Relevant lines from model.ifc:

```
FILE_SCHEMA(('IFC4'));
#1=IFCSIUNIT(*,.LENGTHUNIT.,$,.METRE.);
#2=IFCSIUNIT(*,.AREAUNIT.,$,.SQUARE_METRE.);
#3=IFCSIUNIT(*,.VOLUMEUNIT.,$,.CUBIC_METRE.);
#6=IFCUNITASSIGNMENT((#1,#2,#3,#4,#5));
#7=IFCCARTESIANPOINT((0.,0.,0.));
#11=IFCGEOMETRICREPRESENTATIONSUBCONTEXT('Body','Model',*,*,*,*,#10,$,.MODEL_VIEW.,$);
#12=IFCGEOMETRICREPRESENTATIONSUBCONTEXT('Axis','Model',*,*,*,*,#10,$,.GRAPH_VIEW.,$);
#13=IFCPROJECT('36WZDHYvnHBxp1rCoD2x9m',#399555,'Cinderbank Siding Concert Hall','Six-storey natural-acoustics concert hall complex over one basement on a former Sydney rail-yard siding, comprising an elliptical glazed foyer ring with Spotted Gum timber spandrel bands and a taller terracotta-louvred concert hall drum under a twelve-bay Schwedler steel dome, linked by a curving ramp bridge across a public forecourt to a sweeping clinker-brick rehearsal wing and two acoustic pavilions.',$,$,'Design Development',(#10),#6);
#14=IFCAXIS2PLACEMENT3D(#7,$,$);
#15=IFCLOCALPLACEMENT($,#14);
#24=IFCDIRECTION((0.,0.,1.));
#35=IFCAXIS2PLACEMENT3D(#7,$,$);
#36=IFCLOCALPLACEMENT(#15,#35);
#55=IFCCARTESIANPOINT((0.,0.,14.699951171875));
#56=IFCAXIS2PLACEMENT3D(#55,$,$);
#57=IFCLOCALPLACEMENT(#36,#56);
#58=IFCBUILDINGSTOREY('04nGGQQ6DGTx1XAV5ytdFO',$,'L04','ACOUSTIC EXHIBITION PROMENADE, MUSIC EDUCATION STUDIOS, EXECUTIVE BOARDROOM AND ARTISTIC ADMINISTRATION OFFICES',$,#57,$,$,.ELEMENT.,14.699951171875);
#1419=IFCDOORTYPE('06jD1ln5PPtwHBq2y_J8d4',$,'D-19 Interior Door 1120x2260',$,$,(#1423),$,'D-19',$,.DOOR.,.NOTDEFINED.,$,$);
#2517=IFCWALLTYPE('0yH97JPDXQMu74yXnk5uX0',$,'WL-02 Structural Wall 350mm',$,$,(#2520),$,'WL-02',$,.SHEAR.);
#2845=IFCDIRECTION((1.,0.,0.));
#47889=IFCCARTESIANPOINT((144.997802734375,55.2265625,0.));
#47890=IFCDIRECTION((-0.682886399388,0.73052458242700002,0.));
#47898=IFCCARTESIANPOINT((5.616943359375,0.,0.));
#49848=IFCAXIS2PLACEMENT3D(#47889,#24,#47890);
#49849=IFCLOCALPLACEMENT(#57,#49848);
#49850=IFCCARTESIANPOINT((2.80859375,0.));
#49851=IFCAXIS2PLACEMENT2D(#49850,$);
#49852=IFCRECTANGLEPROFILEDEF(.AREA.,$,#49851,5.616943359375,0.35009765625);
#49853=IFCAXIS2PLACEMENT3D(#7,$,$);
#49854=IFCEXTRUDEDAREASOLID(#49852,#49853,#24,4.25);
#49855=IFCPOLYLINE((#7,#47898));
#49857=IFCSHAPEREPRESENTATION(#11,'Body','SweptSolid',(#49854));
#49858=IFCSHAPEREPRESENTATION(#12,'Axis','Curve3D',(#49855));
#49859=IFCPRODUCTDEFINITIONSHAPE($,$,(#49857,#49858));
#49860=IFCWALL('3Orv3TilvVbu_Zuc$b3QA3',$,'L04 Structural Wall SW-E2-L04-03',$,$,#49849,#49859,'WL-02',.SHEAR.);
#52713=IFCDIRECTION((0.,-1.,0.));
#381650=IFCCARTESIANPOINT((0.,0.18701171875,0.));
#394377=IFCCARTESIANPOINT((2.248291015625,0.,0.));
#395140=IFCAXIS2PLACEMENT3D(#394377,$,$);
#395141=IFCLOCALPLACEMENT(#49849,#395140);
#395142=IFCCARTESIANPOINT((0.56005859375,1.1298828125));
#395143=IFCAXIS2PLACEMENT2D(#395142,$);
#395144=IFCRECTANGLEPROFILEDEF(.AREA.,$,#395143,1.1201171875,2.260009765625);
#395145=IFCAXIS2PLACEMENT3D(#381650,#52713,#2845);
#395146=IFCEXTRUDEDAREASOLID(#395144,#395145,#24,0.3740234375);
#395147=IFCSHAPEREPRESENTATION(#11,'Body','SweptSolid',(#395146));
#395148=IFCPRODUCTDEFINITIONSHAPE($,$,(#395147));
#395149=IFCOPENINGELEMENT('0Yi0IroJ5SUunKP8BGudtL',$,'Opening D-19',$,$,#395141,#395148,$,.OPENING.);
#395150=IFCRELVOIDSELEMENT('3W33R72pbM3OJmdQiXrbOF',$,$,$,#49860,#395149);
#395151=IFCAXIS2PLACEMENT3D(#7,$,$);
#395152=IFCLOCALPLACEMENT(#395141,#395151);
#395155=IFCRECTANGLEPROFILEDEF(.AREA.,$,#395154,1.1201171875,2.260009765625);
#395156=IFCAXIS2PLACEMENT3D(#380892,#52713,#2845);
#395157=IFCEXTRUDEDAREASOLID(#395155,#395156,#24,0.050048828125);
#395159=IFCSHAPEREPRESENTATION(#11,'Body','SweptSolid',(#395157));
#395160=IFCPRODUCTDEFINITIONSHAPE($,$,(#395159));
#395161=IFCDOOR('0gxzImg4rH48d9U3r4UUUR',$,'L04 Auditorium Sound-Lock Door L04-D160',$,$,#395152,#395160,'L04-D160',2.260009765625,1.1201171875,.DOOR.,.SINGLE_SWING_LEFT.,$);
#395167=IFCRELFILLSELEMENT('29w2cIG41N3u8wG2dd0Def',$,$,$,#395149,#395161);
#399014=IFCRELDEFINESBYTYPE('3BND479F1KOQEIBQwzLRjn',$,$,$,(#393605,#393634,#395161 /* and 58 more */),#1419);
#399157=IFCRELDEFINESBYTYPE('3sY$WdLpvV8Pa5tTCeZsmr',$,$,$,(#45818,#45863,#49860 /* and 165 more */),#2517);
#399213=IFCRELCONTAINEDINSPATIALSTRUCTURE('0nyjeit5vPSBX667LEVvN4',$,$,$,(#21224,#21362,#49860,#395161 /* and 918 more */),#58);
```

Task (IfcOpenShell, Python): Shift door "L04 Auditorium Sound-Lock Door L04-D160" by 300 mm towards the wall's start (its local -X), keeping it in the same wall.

```python
import ifcopenshell
import ifcopenshell.api.geometry
import ifcopenshell.util.placement
import ifcopenshell.util.unit

model = ifcopenshell.open("model.ifc")
unit_scale = ifcopenshell.util.unit.calculate_unit_scale(model)

door = model.by_guid("0gxzImg4rH48d9U3r4UUUR")
opening = door.FillsVoids[0].RelatingOpeningElement
wall = opening.VoidsElements[0].RelatingBuildingElement

wall_matrix = ifcopenshell.util.placement.get_local_placement(wall.ObjectPlacement)
shift = wall_matrix[:3, 0] * -0.3 / unit_scale
before = ifcopenshell.util.placement.get_local_placement(door.ObjectPlacement)[:3, 3].copy()

# The door is placed relative to its opening, so it follows when the opening moves.
matrix = ifcopenshell.util.placement.get_local_placement(opening.ObjectPlacement)
matrix[:3, 3] += shift
ifcopenshell.api.geometry.edit_object_placement(
    model, product=opening, matrix=matrix, is_si=False, should_transform_children=True
)

after = ifcopenshell.util.placement.get_local_placement(door.ObjectPlacement)[:3, 3]
print("door moved by", (after - before).round(3) + 0.0)

model.write("model-out.ifc")
```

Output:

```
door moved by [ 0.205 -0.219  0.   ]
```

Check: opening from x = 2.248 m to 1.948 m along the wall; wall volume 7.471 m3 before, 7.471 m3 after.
